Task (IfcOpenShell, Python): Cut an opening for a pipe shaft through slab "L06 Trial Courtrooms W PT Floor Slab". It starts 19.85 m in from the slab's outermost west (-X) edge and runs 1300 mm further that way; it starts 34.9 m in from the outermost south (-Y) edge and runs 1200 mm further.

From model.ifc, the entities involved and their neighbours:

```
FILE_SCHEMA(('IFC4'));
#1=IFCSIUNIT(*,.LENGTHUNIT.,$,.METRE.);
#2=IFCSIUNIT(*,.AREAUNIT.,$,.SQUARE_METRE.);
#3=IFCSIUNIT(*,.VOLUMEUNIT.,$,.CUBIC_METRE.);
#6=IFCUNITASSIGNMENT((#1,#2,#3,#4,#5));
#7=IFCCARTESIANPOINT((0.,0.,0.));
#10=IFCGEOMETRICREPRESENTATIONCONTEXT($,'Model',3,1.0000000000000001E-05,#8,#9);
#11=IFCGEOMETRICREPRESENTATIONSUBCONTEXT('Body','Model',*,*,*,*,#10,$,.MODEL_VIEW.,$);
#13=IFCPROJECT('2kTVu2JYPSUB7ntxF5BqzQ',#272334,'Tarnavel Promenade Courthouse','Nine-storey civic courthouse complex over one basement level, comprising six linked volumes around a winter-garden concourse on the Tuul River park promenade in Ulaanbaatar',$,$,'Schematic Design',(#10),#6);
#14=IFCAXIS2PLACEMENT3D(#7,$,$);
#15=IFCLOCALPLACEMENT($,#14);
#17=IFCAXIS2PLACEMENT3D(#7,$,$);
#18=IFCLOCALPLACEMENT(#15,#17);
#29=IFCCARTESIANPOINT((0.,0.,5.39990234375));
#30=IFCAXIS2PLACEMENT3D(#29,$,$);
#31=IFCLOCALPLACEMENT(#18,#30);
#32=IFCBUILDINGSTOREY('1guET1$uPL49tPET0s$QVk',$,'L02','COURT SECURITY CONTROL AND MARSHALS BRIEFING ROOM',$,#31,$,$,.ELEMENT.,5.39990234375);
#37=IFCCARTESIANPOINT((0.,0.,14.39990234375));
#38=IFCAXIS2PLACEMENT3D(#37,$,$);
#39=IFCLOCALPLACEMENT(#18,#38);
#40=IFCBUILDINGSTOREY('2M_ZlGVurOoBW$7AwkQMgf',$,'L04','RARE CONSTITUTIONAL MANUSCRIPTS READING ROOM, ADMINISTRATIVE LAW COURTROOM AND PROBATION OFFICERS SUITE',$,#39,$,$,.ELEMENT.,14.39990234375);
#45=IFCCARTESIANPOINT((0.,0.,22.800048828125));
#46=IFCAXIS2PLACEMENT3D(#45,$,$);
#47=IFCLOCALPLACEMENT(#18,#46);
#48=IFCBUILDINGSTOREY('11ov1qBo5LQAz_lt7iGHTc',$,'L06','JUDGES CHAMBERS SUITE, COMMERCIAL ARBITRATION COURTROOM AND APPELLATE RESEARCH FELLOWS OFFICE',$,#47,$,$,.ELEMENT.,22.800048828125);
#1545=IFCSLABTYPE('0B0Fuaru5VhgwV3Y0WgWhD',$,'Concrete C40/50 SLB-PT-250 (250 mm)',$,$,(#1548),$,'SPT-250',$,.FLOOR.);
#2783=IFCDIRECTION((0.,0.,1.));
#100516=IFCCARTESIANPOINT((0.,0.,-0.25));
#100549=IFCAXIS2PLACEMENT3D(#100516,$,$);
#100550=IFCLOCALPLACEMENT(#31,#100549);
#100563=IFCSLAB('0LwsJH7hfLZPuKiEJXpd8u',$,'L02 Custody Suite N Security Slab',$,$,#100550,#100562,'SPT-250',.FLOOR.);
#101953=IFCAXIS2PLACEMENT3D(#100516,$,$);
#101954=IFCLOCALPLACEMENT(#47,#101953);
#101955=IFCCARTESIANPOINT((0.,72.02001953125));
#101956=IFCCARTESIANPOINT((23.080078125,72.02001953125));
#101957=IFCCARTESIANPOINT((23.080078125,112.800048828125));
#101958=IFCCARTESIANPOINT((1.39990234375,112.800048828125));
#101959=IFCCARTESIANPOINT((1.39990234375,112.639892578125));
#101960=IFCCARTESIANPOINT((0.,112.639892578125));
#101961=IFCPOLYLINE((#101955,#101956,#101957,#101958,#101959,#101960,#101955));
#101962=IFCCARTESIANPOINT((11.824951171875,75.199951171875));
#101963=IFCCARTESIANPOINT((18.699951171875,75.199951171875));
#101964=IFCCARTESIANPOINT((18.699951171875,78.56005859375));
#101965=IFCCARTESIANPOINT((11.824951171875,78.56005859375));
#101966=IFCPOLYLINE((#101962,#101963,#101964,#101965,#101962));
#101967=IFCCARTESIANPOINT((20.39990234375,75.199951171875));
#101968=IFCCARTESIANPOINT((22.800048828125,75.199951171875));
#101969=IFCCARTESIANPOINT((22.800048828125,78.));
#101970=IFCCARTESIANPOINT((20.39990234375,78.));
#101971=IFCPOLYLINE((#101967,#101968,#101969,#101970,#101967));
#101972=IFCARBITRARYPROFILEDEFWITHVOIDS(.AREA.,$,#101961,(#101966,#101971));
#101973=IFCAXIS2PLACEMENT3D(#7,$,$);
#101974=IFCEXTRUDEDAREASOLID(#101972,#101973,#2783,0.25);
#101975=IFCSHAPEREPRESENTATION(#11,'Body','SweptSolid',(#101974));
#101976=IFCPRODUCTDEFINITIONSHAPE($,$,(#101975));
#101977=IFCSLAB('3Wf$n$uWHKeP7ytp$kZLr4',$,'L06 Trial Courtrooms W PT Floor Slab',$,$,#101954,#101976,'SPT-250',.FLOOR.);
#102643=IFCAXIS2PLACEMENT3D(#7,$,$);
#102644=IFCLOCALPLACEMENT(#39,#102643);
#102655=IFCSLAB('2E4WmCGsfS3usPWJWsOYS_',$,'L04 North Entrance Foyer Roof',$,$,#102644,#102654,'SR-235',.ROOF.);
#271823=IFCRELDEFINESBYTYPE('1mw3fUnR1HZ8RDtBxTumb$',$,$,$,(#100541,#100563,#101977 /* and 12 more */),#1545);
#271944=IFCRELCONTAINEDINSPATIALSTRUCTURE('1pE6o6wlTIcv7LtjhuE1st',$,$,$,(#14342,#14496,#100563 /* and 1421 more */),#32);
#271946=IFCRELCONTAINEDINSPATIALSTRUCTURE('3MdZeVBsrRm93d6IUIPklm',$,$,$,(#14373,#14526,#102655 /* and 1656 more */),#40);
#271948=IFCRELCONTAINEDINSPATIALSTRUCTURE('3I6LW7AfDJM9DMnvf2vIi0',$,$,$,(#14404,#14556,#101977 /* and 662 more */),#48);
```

```python
import numpy as np
import ifcopenshell
import ifcopenshell.api.feature
import ifcopenshell.api.geometry
import ifcopenshell.api.root
import ifcopenshell.geom
import ifcopenshell.util.placement
import ifcopenshell.util.representation
import ifcopenshell.util.shape
import ifcopenshell.util.unit

model = ifcopenshell.open("model.ifc")
unit_scale = ifcopenshell.util.unit.calculate_unit_scale(model)
settings = ifcopenshell.geom.settings()


def volume(element):
    """Net volume in cubic metres, openings subtracted."""
    shape = ifcopenshell.geom.create_shape(settings, element)
    return ifcopenshell.util.shape.get_volume(shape.geometry)


slab = model.by_guid("3Wf$n$uWHKeP7ytp$kZLr4")
before = volume(slab)

# Extent in the slab's own axes, in metres. The edges named are its -X and -Y sides.
slab_shape = ifcopenshell.geom.create_shape(settings, slab)
vertices = ifcopenshell.util.shape.get_vertices(slab_shape.geometry)
x_min, y_min, bottom = vertices.min(axis=0)
top = vertices[:, 2].max()

opening = ifcopenshell.api.root.create_entity(model, ifc_class="IfcOpeningElement", name="Pipe shaft opening", predefined_type="OPENING")
context = ifcopenshell.util.representation.get_context(model, "Model", "Body", "MODEL_VIEW")
width, depth = 1.3, 1.2
outline = [(0.0, 0.0), (width, 0.0), (width, depth), (0.0, depth), (0.0, 0.0)]
# Overshoot both faces by 50 mm so the cut is clean.
shape = ifcopenshell.api.geometry.add_slab_representation(
    model, context=context, depth=top - bottom + 0.1, polyline=outline
)
ifcopenshell.api.geometry.assign_representation(model, product=opening, representation=shape)

matrix = ifcopenshell.util.placement.get_local_placement(slab.ObjectPlacement)
matrix[:, 3] = matrix @ np.append(np.array([x_min + 19.85, y_min + 34.9, bottom - 0.05]) / unit_scale, 1.0)
ifcopenshell.api.geometry.edit_object_placement(model, product=opening, matrix=matrix, is_si=False)
ifcopenshell.api.feature.add_feature(model, feature=opening, element=slab)

after = volume(slab)

print(f"slab volume {before:.3f} -> {after:.3f} m3")

model.write("model-out.ifc")
```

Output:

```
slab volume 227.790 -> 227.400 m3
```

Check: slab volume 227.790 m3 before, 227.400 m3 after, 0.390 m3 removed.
